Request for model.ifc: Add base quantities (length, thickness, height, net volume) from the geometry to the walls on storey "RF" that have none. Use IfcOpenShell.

First a look at what the model holds.

```python
import ifcopenshell
import ifcopenshell.util.element
import ifcopenshell.util.unit

model = ifcopenshell.open("model.ifc")
print(model.schema)
for unit_type in ("LENGTHUNIT", "AREAUNIT", "VOLUMEUNIT"):
    print(unit_type, ifcopenshell.util.unit.calculate_unit_scale(model, unit_type))
storey = next(s for s in model.by_type("IfcBuildingStorey") if s.Name == "RF")
walls = [e for e in ifcopenshell.util.element.get_decomposition(storey) if e.is_a("IfcWall")]
for e in sorted(walls, key=lambda e: e.id()):
    print(e.id(), e.is_a(), e.Name, list(ifcopenshell.util.element.get_psets(e, qtos_only=True)), sep=" | ")
```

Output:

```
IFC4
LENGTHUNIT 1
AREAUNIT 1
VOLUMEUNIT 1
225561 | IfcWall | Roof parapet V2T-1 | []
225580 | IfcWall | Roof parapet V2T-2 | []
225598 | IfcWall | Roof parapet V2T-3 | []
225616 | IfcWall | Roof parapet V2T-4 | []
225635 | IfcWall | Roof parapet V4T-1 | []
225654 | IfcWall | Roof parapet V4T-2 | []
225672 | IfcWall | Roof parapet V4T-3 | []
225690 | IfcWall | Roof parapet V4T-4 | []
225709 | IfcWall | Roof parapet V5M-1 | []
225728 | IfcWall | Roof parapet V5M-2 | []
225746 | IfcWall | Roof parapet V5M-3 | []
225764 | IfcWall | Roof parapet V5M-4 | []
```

```python
import ifcopenshell
import ifcopenshell.api.pset
import ifcopenshell.geom
import ifcopenshell.util.element
import ifcopenshell.util.shape
import ifcopenshell.util.unit

model = ifcopenshell.open("model.ifc")
unit_scale = ifcopenshell.util.unit.calculate_unit_scale(model)
volume_scale = ifcopenshell.util.unit.calculate_unit_scale(model, "VOLUMEUNIT")
settings = ifcopenshell.geom.settings()

storey = next(s for s in model.by_type("IfcBuildingStorey") if s.Name == "RF")
walls = [e for e in ifcopenshell.util.element.get_decomposition(storey) if e.is_a("IfcWall")]

for e in sorted(walls, key=lambda e: e.id()):
    if ifcopenshell.util.element.get_psets(e, qtos_only=True, should_inherit=False):
        continue
    # Geometry comes back in metres, in the element's own axes.
    shape = ifcopenshell.geom.create_shape(settings, e)
    values = {
        "Length": ifcopenshell.util.shape.get_x(shape.geometry) / unit_scale,
        "Width": ifcopenshell.util.shape.get_y(shape.geometry) / unit_scale,
        "Height": ifcopenshell.util.shape.get_z(shape.geometry) / unit_scale,
        "NetVolume": ifcopenshell.util.shape.get_volume(shape.geometry) / volume_scale,
    }
    qto = ifcopenshell.api.pset.add_qto(model, product=e, name="Qto_WallBaseQuantities")
    ifcopenshell.api.pset.edit_qto(model, qto=qto, properties=values)
    print(e.id(), {k: round(v, 3) for k, v in values.items()})

model.write("model_updated.ifc")
```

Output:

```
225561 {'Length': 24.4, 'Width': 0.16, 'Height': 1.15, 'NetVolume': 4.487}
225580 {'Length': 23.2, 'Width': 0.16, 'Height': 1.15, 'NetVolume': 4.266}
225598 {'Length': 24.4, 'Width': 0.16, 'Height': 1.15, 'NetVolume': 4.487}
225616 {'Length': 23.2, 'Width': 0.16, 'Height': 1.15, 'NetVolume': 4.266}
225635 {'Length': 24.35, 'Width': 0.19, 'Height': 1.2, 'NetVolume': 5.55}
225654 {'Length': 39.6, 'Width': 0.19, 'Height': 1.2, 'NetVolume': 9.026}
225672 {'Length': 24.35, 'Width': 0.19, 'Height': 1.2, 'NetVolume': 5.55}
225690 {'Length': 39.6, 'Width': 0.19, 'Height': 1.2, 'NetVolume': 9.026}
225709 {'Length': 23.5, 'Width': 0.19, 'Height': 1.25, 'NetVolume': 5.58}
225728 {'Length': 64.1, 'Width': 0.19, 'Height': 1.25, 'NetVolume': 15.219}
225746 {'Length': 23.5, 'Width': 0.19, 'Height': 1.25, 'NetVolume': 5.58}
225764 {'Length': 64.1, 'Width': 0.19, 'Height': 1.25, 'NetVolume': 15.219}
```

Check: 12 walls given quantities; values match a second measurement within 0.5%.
